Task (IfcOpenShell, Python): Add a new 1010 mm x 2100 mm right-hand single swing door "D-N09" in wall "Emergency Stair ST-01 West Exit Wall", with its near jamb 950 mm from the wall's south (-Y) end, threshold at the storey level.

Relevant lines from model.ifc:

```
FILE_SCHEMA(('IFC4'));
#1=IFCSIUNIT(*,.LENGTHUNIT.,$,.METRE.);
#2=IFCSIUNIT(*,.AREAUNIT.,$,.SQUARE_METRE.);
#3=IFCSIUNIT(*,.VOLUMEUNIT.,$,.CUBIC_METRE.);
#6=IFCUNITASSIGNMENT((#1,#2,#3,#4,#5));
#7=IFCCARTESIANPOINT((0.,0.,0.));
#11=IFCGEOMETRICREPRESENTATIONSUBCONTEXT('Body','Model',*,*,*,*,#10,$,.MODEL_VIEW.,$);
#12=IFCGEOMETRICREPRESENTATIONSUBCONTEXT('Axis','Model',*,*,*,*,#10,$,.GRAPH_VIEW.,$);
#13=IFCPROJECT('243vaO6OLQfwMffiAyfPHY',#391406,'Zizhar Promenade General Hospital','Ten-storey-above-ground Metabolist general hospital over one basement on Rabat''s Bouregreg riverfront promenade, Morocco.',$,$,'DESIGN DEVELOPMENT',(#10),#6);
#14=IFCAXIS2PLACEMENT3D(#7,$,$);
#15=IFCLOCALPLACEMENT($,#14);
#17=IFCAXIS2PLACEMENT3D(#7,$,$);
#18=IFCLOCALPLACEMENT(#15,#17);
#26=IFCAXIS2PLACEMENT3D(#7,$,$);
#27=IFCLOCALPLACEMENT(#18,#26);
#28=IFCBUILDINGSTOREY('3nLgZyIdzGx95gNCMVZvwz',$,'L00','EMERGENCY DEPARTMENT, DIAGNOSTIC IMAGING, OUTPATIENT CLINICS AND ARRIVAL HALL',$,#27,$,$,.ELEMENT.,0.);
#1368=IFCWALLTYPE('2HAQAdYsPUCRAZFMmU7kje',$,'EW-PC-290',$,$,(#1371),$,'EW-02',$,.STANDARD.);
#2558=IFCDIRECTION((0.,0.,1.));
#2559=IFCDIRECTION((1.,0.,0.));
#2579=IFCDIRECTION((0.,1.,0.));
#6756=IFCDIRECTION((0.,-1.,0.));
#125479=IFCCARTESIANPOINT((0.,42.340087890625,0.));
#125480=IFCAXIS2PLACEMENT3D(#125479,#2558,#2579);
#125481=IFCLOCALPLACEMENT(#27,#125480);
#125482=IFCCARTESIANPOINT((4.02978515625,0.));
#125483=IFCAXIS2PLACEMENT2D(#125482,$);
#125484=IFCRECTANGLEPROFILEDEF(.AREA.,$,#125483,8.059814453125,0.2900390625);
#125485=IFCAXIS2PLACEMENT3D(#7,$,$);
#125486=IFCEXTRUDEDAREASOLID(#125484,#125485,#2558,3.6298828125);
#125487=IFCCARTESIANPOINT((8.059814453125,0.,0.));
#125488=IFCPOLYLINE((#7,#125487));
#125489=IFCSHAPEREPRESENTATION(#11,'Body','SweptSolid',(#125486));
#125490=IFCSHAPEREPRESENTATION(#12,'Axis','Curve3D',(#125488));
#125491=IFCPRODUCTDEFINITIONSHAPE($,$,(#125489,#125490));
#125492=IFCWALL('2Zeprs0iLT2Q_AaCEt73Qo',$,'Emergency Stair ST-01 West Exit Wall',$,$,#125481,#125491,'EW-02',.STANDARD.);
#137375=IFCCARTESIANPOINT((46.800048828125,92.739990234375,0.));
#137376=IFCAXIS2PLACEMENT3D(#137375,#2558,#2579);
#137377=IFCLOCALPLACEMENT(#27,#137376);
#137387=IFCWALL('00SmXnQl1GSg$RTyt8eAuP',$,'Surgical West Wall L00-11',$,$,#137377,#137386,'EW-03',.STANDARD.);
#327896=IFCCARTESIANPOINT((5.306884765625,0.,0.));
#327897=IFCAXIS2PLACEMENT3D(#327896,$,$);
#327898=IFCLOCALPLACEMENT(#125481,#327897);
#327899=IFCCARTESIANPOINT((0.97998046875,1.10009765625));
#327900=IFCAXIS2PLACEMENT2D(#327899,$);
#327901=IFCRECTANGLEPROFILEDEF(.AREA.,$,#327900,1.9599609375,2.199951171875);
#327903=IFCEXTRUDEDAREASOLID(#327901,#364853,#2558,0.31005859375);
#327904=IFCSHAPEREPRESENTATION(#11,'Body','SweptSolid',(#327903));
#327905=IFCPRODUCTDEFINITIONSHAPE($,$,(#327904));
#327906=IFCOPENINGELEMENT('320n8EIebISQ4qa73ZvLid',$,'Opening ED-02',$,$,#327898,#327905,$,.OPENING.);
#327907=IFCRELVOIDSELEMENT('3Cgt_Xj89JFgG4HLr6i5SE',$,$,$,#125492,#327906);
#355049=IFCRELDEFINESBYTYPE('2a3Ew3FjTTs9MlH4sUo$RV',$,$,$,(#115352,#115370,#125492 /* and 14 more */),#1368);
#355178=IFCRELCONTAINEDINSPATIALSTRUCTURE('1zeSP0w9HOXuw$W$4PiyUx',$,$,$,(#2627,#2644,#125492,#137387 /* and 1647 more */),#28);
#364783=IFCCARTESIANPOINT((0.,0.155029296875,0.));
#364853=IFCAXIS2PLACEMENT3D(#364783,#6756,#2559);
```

```python
import numpy as np
import ifcopenshell
import ifcopenshell.api.feature
import ifcopenshell.api.geometry
import ifcopenshell.api.root
import ifcopenshell.api.spatial
import ifcopenshell.geom
import ifcopenshell.util.element
import ifcopenshell.util.placement
import ifcopenshell.util.representation
import ifcopenshell.util.shape
import ifcopenshell.util.unit

model = ifcopenshell.open("model.ifc")
unit_scale = ifcopenshell.util.unit.calculate_unit_scale(model)
settings = ifcopenshell.geom.settings()


def volume(element):
    """Net volume in cubic metres, openings subtracted."""
    shape = ifcopenshell.geom.create_shape(settings, element)
    return ifcopenshell.util.shape.get_volume(shape.geometry)


wall = model.by_id(125492)
storey = ifcopenshell.util.element.get_container(wall, ifc_class="IfcBuildingStorey")
context = ifcopenshell.util.representation.get_context(model, "Model", "Body", "MODEL_VIEW")
before = volume(wall)

width, height, from_end, sill = 1.01, 2.1, 0.95, 0.0  # metres

# The wall runs along its own X axis, and the end named is its -X end.
wall_shape = ifcopenshell.geom.create_shape(settings, wall)
x, y, z = ifcopenshell.util.shape.get_vertices(wall_shape.geometry).T
start = x.min() + from_end
face, thickness = float(y.min()), float(y.max() - y.min())
wall_matrix = ifcopenshell.util.placement.get_local_placement(wall.ObjectPlacement)
level = ifcopenshell.util.placement.get_local_placement(storey.ObjectPlacement)[2, 3]


def in_wall(x, y):
    """Placement at x, y metres in the wall's axes, at sill height."""
    matrix = wall_matrix.copy()
    matrix[:, 3] = wall_matrix @ np.array([x / unit_scale, y / unit_scale, 0.0, 1.0])
    matrix[2, 3] = level + sill / unit_scale
    return matrix


# Opening: a box that overshoots both wall faces by 50 mm.
opening = ifcopenshell.api.root.create_entity(model, ifc_class="IfcOpeningElement", predefined_type="OPENING")
box = ifcopenshell.api.geometry.add_wall_representation(
    model, context=context, length=width, height=height, thickness=thickness + 0.1
)
ifcopenshell.api.geometry.assign_representation(model, product=opening, representation=box)
ifcopenshell.api.geometry.edit_object_placement(model, product=opening, matrix=in_wall(start, face - 0.05), is_si=False)
ifcopenshell.api.feature.add_feature(model, feature=opening, element=wall)

door = ifcopenshell.api.root.create_entity(model, ifc_class="IfcDoor", name="D-N09", predefined_type="DOOR")
door.OverallWidth, door.OverallHeight = width / unit_scale, height / unit_scale
door.OperationType = "SINGLE_SWING_RIGHT"
body = ifcopenshell.api.geometry.add_door_representation(
    model,
    context=context,
    overall_width=door.OverallWidth,
    overall_height=door.OverallHeight,
    operation_type="SINGLE_SWING_RIGHT",
    lining_properties={"LiningDepth": thickness / unit_scale, "ThresholdDepth": thickness / unit_scale},
)
ifcopenshell.api.geometry.assign_representation(model, product=door, representation=body)
ifcopenshell.api.spatial.assign_container(model, products=[door], relating_structure=storey)
ifcopenshell.api.feature.add_filling(model, opening=opening, element=door)

# The lining spans the wall, so the door starts at the wall face.
ifcopenshell.api.geometry.edit_object_placement(model, product=door, matrix=in_wall(start, face), is_si=False)

after = volume(wall)

print(f"wall volume {before:.3f} -> {after:.3f} m3")

model.write("model_edited.ifc")
```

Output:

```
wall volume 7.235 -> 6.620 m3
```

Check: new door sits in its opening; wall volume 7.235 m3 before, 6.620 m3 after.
